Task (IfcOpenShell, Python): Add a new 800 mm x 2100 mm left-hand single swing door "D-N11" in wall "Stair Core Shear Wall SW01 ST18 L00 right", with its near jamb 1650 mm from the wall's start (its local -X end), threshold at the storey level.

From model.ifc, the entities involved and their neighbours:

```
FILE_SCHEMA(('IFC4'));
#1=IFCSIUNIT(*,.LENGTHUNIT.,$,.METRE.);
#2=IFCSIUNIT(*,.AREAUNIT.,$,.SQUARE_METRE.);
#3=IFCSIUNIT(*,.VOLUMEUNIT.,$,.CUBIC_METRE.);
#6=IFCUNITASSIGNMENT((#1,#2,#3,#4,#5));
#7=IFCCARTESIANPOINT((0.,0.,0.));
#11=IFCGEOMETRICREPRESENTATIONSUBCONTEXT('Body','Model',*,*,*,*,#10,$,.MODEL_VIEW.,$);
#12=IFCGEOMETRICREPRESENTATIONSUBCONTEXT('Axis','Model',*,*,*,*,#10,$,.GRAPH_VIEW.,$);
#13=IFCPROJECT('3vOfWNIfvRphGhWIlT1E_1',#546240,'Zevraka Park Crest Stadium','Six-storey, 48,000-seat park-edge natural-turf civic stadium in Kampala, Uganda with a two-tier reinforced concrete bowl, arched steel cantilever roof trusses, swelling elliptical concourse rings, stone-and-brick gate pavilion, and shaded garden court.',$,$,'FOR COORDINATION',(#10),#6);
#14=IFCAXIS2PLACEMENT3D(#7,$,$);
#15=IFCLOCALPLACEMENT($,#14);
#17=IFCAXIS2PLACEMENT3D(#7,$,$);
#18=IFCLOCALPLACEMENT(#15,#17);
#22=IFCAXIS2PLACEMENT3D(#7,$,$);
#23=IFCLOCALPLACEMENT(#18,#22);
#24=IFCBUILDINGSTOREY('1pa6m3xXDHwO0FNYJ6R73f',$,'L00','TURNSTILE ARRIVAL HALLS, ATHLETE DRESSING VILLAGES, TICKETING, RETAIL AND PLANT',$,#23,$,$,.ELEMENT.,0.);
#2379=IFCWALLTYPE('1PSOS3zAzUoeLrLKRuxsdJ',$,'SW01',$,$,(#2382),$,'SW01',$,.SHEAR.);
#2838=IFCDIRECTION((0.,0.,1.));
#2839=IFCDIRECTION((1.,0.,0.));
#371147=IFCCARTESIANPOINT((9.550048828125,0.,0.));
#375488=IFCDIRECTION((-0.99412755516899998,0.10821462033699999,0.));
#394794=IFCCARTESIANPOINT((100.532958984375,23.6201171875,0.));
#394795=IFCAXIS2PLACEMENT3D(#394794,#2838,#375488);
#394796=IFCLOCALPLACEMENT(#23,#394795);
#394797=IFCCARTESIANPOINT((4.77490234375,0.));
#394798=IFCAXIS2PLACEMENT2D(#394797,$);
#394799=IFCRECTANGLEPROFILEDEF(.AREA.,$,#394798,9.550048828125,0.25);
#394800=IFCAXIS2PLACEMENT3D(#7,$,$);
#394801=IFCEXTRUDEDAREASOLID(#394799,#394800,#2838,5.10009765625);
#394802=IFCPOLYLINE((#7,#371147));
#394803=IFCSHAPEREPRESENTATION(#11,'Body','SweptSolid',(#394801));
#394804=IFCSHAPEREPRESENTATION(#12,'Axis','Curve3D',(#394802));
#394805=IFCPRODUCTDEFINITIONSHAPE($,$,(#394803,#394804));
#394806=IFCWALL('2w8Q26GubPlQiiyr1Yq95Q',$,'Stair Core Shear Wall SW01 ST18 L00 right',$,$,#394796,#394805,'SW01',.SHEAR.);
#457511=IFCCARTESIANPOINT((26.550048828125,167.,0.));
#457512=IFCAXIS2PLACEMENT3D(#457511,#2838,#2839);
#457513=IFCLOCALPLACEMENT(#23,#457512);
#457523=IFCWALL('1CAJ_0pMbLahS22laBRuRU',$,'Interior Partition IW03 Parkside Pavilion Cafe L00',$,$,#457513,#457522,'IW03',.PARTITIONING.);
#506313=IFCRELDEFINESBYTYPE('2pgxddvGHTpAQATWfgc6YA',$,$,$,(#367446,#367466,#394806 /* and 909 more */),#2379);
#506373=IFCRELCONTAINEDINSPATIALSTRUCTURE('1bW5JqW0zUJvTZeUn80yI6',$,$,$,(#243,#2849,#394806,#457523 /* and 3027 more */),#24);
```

```python
import numpy as np
import ifcopenshell
import ifcopenshell.api.feature
import ifcopenshell.api.geometry
import ifcopenshell.api.root
import ifcopenshell.api.spatial
import ifcopenshell.geom
import ifcopenshell.util.element
import ifcopenshell.util.placement
import ifcopenshell.util.representation
import ifcopenshell.util.shape
import ifcopenshell.util.unit

model = ifcopenshell.open("model.ifc")
unit_scale = ifcopenshell.util.unit.calculate_unit_scale(model)
settings = ifcopenshell.geom.settings()


def volume(element):
    """Net volume in cubic metres, openings subtracted."""
    shape = ifcopenshell.geom.create_shape(settings, element)
    return ifcopenshell.util.shape.get_volume(shape.geometry)


wall = model.by_guid("2w8Q26GubPlQiiyr1Yq95Q")
storey = ifcopenshell.util.element.get_container(wall, ifc_class="IfcBuildingStorey")
context = ifcopenshell.util.representation.get_context(model, "Model", "Body", "MODEL_VIEW")
before = volume(wall)

width, height, from_end, sill = 0.8, 2.1, 1.65, 0.0  # metres

# The wall runs along its own X axis, and the end named is its -X end.
wall_shape = ifcopenshell.geom.create_shape(settings, wall)
x, y, z = ifcopenshell.util.shape.get_vertices(wall_shape.geometry).T
start = x.min() + from_end
face, thickness = float(y.min()), float(y.max() - y.min())
wall_matrix = ifcopenshell.util.placement.get_local_placement(wall.ObjectPlacement)
level = ifcopenshell.util.placement.get_local_placement(storey.ObjectPlacement)[2, 3]


def in_wall(x, y):
    """Placement at x, y metres in the wall's axes, at sill height."""
    matrix = wall_matrix.copy()
    matrix[:, 3] = wall_matrix @ np.array([x / unit_scale, y / unit_scale, 0.0, 1.0])
    matrix[2, 3] = level + sill / unit_scale
    return matrix


# Opening: a box that overshoots both wall faces by 50 mm.
opening = ifcopenshell.api.root.create_entity(model, ifc_class="IfcOpeningElement", predefined_type="OPENING")
box = ifcopenshell.api.geometry.add_wall_representation(
    model, context=context, length=width, height=height, thickness=thickness + 0.1
)
ifcopenshell.api.geometry.assign_representation(model, product=opening, representation=box)
ifcopenshell.api.geometry.edit_object_placement(model, product=opening, matrix=in_wall(start, face - 0.05), is_si=False)
ifcopenshell.api.feature.add_feature(model, feature=opening, element=wall)

door = ifcopenshell.api.root.create_entity(model, ifc_class="IfcDoor", name="D-N11", predefined_type="DOOR")
door.OverallWidth, door.OverallHeight = width / unit_scale, height / unit_scale
door.OperationType = "SINGLE_SWING_LEFT"
body = ifcopenshell.api.geometry.add_door_representation(
    model,
    context=context,
    overall_width=door.OverallWidth,
    overall_height=door.OverallHeight,
    operation_type="SINGLE_SWING_LEFT",
    lining_properties={"LiningDepth": thickness / unit_scale, "ThresholdDepth": thickness / unit_scale},
)
ifcopenshell.api.geometry.assign_representation(model, product=door, representation=body)
ifcopenshell.api.spatial.assign_container(model, products=[door], relating_structure=storey)
ifcopenshell.api.feature.add_filling(model, opening=opening, element=door)

# The lining spans the wall, so the door starts at the wall face.
ifcopenshell.api.geometry.edit_object_placement(model, product=door, matrix=in_wall(start, face), is_si=False)

after = volume(wall)

print(f"wall volume {before:.3f} -> {after:.3f} m3")

model.write("model-out.ifc")
```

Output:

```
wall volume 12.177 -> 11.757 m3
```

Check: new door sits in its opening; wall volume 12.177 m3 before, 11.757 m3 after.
